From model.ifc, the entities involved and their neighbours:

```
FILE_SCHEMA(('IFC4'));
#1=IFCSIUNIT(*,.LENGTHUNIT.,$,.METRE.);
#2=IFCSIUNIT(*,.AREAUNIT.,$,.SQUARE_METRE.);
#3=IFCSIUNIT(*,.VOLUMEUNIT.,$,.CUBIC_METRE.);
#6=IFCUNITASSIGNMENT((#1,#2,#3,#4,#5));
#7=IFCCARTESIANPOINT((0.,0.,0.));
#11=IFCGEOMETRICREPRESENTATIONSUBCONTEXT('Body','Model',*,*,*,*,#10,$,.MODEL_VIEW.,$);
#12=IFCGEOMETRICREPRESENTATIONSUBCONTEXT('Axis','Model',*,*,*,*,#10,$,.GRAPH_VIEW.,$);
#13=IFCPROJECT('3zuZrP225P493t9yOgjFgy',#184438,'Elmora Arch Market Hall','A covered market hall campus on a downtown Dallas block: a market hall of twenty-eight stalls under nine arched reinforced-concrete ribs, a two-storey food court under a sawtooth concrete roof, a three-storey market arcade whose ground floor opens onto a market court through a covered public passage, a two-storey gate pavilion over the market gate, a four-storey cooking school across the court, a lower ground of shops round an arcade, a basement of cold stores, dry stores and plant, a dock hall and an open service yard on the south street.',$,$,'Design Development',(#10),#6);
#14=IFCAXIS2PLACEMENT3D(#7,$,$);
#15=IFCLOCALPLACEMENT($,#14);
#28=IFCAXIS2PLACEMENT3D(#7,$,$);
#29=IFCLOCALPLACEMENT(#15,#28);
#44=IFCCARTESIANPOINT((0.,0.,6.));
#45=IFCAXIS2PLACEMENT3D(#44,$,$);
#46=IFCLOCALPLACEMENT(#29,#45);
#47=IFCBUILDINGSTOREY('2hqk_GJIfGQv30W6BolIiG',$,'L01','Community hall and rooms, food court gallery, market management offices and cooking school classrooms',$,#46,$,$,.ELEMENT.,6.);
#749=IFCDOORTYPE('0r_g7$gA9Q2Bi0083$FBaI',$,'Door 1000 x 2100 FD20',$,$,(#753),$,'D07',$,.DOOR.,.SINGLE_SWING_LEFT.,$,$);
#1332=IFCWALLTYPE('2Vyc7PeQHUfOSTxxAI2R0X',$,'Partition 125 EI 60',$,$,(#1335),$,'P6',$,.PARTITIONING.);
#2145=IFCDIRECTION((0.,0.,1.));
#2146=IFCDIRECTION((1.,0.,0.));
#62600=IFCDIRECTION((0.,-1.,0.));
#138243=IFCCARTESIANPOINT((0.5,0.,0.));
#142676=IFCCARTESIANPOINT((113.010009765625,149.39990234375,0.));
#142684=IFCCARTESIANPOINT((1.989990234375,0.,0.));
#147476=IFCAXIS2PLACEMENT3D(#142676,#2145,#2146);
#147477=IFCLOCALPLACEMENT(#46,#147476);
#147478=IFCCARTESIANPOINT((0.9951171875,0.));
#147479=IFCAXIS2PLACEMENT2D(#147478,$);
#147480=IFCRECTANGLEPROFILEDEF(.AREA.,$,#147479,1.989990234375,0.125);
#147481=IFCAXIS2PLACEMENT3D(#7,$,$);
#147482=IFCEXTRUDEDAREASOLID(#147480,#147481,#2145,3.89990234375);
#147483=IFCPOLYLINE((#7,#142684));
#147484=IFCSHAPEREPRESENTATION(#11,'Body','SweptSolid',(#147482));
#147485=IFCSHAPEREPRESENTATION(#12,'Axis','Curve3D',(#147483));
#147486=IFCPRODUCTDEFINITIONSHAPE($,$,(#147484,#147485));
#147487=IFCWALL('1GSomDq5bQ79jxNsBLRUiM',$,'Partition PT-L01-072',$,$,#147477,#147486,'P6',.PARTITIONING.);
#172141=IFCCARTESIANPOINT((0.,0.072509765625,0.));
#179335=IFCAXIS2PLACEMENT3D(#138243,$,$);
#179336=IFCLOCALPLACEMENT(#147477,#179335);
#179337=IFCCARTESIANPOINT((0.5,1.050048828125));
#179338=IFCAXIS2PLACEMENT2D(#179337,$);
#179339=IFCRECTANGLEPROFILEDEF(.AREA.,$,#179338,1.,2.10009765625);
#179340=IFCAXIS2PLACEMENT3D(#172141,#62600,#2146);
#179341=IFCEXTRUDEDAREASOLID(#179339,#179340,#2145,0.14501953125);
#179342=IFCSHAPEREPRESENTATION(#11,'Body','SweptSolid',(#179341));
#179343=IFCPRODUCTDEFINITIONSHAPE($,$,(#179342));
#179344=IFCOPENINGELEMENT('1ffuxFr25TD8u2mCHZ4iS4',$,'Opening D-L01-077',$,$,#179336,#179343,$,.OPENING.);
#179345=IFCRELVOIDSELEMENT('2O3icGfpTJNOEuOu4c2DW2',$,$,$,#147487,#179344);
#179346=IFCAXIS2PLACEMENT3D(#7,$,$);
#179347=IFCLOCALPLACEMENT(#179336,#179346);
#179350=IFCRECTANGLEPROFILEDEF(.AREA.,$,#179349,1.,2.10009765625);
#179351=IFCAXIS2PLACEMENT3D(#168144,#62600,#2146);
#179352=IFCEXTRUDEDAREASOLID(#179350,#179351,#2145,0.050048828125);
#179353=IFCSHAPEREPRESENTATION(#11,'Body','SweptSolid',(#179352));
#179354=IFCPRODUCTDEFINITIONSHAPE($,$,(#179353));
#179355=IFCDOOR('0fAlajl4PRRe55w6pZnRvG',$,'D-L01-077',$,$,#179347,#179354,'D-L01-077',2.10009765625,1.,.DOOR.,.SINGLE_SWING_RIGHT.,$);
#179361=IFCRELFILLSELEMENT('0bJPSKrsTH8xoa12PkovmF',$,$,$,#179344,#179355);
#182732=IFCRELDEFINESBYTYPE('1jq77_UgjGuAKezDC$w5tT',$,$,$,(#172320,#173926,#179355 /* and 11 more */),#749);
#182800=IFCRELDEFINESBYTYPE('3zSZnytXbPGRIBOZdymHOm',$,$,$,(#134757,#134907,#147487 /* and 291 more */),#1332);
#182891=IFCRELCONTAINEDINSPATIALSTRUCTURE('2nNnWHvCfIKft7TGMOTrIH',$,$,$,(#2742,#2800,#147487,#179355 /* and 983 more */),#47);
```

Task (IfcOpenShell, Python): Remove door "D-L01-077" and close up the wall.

```python
import ifcopenshell
import ifcopenshell.api.feature
import ifcopenshell.api.root
import ifcopenshell.geom
import ifcopenshell.util.shape

model = ifcopenshell.open("model.ifc")
settings = ifcopenshell.geom.settings()


def volume(element):
    """Net volume in cubic metres, openings subtracted."""
    shape = ifcopenshell.geom.create_shape(settings, element)
    return ifcopenshell.util.shape.get_volume(shape.geometry)


door = model.by_guid("0fAlajl4PRRe55w6pZnRvG")
opening = door.FillsVoids[0].RelatingOpeningElement
wall = opening.VoidsElements[0].RelatingBuildingElement
before = volume(wall)

ifcopenshell.api.root.remove_product(model, product=door)
ifcopenshell.api.feature.remove_feature(model, feature=opening)

after = volume(wall)

print(f"wall volume {before:.3f} -> {after:.3f} m3")

model.write("model-out.ifc")
```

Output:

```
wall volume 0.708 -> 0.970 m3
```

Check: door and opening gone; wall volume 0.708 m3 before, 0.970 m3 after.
